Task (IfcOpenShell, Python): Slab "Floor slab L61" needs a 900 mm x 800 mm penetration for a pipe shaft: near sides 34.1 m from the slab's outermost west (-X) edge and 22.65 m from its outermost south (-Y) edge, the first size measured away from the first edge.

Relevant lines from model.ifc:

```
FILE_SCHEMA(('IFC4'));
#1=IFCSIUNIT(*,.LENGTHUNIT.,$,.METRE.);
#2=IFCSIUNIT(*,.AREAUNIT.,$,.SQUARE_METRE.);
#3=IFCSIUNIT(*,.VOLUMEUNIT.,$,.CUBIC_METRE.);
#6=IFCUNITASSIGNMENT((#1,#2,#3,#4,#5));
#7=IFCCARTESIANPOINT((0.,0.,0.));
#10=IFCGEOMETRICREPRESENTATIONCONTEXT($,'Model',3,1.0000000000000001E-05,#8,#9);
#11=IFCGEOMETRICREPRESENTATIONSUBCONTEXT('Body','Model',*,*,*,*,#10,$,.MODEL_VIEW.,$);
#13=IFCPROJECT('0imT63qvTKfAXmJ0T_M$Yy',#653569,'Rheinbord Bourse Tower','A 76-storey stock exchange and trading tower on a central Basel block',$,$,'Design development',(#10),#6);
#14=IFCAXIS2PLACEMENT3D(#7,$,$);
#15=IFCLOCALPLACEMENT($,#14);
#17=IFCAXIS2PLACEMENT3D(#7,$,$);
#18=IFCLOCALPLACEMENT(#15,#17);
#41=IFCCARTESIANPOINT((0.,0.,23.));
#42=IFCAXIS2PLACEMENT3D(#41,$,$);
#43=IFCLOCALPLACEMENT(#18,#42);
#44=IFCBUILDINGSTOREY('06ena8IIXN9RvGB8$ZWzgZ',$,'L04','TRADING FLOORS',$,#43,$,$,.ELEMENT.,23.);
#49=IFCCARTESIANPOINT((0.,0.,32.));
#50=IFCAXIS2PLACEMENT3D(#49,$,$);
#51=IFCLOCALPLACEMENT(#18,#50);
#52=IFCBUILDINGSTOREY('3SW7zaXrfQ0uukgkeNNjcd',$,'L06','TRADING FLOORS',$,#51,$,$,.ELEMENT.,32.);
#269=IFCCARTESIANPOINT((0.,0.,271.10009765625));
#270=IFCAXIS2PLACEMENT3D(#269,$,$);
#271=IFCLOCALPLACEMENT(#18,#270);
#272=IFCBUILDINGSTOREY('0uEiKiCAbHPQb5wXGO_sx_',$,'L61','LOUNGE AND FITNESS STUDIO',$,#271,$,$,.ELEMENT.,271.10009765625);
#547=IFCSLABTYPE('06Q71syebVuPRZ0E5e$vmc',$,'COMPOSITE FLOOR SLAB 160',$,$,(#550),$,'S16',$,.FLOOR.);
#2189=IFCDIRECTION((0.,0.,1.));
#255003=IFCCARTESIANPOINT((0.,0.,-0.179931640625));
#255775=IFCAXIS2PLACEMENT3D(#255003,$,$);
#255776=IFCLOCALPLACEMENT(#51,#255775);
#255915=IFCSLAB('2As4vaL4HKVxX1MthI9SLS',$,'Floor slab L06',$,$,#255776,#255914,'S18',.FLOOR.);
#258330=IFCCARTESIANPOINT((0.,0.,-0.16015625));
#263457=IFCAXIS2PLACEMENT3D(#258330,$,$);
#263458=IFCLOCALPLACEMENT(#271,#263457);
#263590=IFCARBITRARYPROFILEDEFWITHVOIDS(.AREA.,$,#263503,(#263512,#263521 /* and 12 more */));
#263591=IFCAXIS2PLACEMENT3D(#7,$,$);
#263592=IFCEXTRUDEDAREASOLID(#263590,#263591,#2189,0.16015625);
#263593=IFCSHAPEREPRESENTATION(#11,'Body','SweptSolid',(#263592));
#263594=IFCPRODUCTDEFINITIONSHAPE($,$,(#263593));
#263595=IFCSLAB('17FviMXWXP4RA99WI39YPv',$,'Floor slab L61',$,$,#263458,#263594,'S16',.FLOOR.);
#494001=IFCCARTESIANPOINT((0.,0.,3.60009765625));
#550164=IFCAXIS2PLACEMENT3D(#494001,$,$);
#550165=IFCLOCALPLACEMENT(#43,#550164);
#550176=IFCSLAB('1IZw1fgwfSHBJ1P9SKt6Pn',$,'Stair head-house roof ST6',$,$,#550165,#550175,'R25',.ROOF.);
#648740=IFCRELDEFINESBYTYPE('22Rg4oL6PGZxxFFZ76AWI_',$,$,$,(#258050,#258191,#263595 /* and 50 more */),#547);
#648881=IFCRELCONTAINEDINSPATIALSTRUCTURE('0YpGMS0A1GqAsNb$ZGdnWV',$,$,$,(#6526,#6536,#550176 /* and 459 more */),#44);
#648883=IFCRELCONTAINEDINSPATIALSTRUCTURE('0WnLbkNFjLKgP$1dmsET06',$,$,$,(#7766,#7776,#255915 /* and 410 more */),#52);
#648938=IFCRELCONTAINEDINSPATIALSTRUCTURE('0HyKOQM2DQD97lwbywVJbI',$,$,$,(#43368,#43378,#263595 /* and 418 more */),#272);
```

```python
import numpy as np
import ifcopenshell
import ifcopenshell.api.feature
import ifcopenshell.api.geometry
import ifcopenshell.api.root
import ifcopenshell.geom
import ifcopenshell.util.placement
import ifcopenshell.util.representation
import ifcopenshell.util.shape
import ifcopenshell.util.unit

model = ifcopenshell.open("model.ifc")
unit_scale = ifcopenshell.util.unit.calculate_unit_scale(model)
settings = ifcopenshell.geom.settings()


def volume(element):
    """Net volume in cubic metres, openings subtracted."""
    shape = ifcopenshell.geom.create_shape(settings, element)
    return ifcopenshell.util.shape.get_volume(shape.geometry)


slab = model.by_guid("17FviMXWXP4RA99WI39YPv")
before = volume(slab)

# Extent in the slab's own axes, in metres. The edges named are its -X and -Y sides.
slab_shape = ifcopenshell.geom.create_shape(settings, slab)
vertices = ifcopenshell.util.shape.get_vertices(slab_shape.geometry)
x_min, y_min, bottom = vertices.min(axis=0)
top = vertices[:, 2].max()

opening = ifcopenshell.api.root.create_entity(model, ifc_class="IfcOpeningElement", name="Pipe shaft opening", predefined_type="OPENING")
context = ifcopenshell.util.representation.get_context(model, "Model", "Body", "MODEL_VIEW")
width, depth = 0.9, 0.8
outline = [(0.0, 0.0), (width, 0.0), (width, depth), (0.0, depth), (0.0, 0.0)]
# Overshoot both faces by 50 mm so the cut is clean.
shape = ifcopenshell.api.geometry.add_slab_representation(
    model, context=context, depth=top - bottom + 0.1, polyline=outline
)
ifcopenshell.api.geometry.assign_representation(model, product=opening, representation=shape)

matrix = ifcopenshell.util.placement.get_local_placement(slab.ObjectPlacement)
matrix[:, 3] = matrix @ np.append(np.array([x_min + 34.1, y_min + 22.65, bottom - 0.05]) / unit_scale, 1.0)
ifcopenshell.api.geometry.edit_object_placement(model, product=opening, matrix=matrix, is_si=False)
ifcopenshell.api.feature.add_feature(model, feature=opening, element=slab)

after = volume(slab)

print(f"slab volume {before:.3f} -> {after:.3f} m3")

model.write("model-out.ifc")
```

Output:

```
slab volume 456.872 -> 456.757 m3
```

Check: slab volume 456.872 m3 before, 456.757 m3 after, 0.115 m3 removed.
